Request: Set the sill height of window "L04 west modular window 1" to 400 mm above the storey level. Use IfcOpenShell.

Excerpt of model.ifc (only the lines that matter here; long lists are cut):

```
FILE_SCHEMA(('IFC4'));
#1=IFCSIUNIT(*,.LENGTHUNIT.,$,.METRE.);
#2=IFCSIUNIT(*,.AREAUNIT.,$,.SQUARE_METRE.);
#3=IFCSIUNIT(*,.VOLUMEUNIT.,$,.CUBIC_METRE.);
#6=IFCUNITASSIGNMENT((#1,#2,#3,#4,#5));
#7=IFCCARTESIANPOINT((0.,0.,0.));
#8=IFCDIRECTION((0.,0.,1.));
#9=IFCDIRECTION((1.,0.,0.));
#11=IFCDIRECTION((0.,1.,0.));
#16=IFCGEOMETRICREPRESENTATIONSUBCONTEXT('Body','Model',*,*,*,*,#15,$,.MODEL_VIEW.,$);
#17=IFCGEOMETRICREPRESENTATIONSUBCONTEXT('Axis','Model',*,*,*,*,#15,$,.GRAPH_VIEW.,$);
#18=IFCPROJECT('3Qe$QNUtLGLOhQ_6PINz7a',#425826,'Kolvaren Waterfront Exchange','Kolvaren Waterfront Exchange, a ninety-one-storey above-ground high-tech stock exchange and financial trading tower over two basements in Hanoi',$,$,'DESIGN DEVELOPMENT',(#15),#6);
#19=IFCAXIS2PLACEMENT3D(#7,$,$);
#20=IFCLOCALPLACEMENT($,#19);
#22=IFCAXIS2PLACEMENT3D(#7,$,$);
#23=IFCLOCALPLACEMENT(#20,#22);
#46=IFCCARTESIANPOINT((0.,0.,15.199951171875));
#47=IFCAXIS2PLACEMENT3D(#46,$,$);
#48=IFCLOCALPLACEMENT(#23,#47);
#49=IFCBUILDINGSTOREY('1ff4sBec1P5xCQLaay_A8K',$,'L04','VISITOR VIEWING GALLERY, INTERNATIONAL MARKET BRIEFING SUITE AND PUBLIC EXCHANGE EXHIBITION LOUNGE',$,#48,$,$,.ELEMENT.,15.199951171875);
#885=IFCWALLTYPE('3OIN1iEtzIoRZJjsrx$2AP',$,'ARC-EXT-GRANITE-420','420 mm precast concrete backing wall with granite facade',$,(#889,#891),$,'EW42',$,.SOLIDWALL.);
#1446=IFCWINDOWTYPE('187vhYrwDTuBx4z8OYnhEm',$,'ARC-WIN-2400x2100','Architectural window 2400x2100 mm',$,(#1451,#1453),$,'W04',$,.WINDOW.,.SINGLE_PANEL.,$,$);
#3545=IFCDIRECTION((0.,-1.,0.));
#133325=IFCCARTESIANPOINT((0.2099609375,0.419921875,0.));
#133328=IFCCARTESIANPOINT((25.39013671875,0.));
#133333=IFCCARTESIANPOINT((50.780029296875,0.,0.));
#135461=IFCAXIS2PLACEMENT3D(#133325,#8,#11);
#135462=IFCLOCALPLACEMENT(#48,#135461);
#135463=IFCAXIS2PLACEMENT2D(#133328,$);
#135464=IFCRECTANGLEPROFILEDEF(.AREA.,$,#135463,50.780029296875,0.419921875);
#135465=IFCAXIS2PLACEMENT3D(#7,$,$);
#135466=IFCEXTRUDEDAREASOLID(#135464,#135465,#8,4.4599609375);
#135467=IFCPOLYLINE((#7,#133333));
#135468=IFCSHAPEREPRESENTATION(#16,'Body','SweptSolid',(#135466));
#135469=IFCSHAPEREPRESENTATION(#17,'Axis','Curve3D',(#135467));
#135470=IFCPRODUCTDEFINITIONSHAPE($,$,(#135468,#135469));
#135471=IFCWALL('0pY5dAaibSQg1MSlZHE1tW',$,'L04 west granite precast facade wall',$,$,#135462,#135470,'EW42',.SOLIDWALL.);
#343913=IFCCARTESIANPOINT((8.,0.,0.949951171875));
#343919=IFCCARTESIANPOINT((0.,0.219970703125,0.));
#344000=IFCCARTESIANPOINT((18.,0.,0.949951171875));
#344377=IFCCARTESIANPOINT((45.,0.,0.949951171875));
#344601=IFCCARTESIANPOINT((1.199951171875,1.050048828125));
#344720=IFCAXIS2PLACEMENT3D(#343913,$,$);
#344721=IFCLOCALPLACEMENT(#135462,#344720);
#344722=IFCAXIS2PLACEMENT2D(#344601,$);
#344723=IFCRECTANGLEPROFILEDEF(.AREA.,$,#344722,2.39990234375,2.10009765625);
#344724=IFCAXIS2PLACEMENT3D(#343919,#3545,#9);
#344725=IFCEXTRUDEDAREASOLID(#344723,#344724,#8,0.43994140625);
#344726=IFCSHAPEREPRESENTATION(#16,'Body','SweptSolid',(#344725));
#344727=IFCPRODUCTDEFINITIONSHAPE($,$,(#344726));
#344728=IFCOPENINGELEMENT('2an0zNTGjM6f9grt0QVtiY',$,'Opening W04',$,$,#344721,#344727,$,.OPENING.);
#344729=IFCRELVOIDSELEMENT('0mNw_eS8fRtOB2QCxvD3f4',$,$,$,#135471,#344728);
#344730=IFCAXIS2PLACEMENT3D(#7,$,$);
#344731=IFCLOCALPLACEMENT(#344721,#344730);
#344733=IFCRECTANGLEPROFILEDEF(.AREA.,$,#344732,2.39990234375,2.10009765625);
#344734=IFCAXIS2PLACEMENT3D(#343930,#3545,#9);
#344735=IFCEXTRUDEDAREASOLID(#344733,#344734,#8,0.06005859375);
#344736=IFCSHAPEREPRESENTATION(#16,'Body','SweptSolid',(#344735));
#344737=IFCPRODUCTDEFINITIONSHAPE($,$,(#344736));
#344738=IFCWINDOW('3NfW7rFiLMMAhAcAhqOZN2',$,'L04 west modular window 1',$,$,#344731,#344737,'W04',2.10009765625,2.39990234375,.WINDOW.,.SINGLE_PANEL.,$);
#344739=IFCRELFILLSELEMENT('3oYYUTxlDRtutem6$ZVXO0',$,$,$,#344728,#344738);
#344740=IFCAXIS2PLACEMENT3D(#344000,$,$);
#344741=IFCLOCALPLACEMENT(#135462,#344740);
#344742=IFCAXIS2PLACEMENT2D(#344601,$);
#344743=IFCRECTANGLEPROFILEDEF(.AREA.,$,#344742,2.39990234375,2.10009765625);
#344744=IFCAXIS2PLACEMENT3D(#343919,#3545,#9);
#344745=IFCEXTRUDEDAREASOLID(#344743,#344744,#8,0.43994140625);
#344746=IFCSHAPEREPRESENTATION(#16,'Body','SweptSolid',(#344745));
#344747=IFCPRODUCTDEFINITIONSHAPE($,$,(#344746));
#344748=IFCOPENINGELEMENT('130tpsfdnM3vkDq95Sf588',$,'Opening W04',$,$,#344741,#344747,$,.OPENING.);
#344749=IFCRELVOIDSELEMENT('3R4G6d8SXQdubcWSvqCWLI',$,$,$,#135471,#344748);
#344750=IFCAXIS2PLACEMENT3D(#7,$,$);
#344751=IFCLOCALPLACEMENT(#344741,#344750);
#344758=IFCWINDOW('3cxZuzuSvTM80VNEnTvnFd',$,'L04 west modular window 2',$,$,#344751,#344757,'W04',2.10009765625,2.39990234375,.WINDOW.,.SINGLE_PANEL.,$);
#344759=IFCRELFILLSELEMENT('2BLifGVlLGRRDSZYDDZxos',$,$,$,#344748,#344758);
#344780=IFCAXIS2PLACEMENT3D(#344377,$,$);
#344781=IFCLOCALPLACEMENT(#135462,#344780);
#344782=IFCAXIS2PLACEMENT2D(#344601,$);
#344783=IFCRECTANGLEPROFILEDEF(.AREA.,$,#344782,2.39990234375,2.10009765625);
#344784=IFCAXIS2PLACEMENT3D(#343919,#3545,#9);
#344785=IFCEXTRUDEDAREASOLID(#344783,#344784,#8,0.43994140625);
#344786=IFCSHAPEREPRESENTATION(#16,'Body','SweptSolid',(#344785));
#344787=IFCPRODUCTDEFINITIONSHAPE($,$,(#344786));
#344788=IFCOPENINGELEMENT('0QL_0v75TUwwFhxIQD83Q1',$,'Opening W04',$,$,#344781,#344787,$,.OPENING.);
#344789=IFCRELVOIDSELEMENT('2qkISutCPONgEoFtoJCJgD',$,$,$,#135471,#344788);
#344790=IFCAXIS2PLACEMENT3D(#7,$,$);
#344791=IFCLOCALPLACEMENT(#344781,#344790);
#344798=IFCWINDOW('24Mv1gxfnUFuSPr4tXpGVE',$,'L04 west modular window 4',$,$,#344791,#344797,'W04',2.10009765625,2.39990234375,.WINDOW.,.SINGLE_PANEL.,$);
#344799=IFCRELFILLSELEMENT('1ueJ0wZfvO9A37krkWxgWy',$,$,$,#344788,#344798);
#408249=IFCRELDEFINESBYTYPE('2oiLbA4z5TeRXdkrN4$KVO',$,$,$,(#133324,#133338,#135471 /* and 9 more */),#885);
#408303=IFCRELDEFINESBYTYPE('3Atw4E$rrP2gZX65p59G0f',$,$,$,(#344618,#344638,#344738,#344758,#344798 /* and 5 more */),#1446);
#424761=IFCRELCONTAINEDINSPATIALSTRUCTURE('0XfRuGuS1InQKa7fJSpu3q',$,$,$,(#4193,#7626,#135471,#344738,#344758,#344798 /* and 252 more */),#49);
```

```python
import numpy as np
import ifcopenshell
import ifcopenshell.api.geometry
import ifcopenshell.geom
import ifcopenshell.util.element
import ifcopenshell.util.placement
import ifcopenshell.util.shape
import ifcopenshell.util.unit

model = ifcopenshell.open("model.ifc")
unit_scale = ifcopenshell.util.unit.calculate_unit_scale(model)

window = model.by_id(344738)
opening = window.FillsVoids[0].RelatingOpeningElement
storey = ifcopenshell.util.element.get_container(window, ifc_class="IfcBuildingStorey")
level = ifcopenshell.util.placement.get_local_placement(storey.ObjectPlacement)[2, 3]

# The opening's origin need not be at the sill, so measure its lowest point.
shape = ifcopenshell.geom.create_shape(ifcopenshell.geom.settings(), opening)
bottom = ifcopenshell.util.shape.get_shape_bottom_elevation(shape, shape.geometry) / unit_scale
dz = level + 0.4 / unit_scale - bottom

shift = np.array([0.0, 0.0, dz])
# The window is placed relative to its opening, so it follows when the opening moves.
matrix = ifcopenshell.util.placement.get_local_placement(opening.ObjectPlacement)
matrix[:3, 3] += shift
ifcopenshell.api.geometry.edit_object_placement(
    model, product=opening, matrix=matrix, is_si=False, should_transform_children=True
)

print(f"moved by {dz * unit_scale:+.3f} m")

model.write("model_rev.ifc")
```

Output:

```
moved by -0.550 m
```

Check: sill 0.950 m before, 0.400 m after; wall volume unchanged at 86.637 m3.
